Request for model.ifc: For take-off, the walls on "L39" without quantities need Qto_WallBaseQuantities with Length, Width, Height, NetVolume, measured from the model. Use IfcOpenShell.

First a look at what the model holds.

```python
import ifcopenshell
import ifcopenshell.util.element
import ifcopenshell.util.unit

model = ifcopenshell.open("model.ifc")
print(model.schema)
for unit_type in ("LENGTHUNIT", "AREAUNIT", "VOLUMEUNIT"):
    print(unit_type, ifcopenshell.util.unit.calculate_unit_scale(model, unit_type))
storey = next(s for s in model.by_type("IfcBuildingStorey") if s.Name == "L39")
walls = [e for e in ifcopenshell.util.element.get_decomposition(storey) if e.is_a("IfcWall")]
for e in sorted(walls, key=lambda e: e.id()):
    print(e.id(), e.is_a(), e.Name, list(ifcopenshell.util.element.get_psets(e, qtos_only=True)), sep=" | ")
```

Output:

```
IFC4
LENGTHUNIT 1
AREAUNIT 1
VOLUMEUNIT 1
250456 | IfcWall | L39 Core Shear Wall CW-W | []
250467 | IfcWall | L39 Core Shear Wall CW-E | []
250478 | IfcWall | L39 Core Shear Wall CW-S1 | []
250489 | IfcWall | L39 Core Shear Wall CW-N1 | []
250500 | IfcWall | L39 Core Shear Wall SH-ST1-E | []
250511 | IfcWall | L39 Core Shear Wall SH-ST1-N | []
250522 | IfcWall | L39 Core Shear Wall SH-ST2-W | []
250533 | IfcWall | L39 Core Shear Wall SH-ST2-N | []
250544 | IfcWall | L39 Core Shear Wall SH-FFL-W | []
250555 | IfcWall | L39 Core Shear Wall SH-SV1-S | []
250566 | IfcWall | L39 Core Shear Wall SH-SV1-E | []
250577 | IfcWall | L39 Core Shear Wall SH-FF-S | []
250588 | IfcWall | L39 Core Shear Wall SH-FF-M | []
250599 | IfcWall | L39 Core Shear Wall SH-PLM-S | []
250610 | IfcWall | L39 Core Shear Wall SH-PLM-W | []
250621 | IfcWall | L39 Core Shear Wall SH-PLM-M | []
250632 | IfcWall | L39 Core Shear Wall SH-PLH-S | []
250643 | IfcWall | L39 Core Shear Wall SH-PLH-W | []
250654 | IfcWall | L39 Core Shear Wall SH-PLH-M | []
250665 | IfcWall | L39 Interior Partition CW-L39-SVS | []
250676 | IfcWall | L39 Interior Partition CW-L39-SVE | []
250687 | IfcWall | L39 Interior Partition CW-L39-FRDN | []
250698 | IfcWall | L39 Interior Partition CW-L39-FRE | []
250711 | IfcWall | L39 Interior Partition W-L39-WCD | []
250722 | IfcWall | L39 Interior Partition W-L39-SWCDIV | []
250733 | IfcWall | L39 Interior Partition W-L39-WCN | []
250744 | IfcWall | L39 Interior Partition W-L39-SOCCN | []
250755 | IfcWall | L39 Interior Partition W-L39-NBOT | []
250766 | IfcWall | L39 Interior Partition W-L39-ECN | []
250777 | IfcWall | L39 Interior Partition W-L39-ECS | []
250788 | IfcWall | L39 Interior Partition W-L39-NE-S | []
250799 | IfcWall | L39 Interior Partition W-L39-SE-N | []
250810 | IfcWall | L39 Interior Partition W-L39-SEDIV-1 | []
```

```python
import ifcopenshell
import ifcopenshell.api.pset
import ifcopenshell.geom
import ifcopenshell.util.element
import ifcopenshell.util.shape
import ifcopenshell.util.unit

model = ifcopenshell.open("model.ifc")
unit_scale = ifcopenshell.util.unit.calculate_unit_scale(model)
volume_scale = ifcopenshell.util.unit.calculate_unit_scale(model, "VOLUMEUNIT")
settings = ifcopenshell.geom.settings()

storey = next(s for s in model.by_type("IfcBuildingStorey") if s.Name == "L39")
walls = [e for e in ifcopenshell.util.element.get_decomposition(storey) if e.is_a("IfcWall")]

for e in sorted(walls, key=lambda e: e.id()):
    if ifcopenshell.util.element.get_psets(e, qtos_only=True, should_inherit=False):
        continue
    # Geometry comes back in metres, in the element's own axes.
    shape = ifcopenshell.geom.create_shape(settings, e)
    values = {
        "Length": ifcopenshell.util.shape.get_x(shape.geometry) / unit_scale,
        "Width": ifcopenshell.util.shape.get_y(shape.geometry) / unit_scale,
        "Height": ifcopenshell.util.shape.get_z(shape.geometry) / unit_scale,
        "NetVolume": ifcopenshell.util.shape.get_volume(shape.geometry) / volume_scale,
    }
    qto = ifcopenshell.api.pset.add_qto(model, product=e, name="Qto_WallBaseQuantities")
    ifcopenshell.api.pset.edit_qto(model, qto=qto, properties=values)
    print(e.id(), {k: round(v, 3) for k, v in values.items()})

model.write("model_updated.ifc")
```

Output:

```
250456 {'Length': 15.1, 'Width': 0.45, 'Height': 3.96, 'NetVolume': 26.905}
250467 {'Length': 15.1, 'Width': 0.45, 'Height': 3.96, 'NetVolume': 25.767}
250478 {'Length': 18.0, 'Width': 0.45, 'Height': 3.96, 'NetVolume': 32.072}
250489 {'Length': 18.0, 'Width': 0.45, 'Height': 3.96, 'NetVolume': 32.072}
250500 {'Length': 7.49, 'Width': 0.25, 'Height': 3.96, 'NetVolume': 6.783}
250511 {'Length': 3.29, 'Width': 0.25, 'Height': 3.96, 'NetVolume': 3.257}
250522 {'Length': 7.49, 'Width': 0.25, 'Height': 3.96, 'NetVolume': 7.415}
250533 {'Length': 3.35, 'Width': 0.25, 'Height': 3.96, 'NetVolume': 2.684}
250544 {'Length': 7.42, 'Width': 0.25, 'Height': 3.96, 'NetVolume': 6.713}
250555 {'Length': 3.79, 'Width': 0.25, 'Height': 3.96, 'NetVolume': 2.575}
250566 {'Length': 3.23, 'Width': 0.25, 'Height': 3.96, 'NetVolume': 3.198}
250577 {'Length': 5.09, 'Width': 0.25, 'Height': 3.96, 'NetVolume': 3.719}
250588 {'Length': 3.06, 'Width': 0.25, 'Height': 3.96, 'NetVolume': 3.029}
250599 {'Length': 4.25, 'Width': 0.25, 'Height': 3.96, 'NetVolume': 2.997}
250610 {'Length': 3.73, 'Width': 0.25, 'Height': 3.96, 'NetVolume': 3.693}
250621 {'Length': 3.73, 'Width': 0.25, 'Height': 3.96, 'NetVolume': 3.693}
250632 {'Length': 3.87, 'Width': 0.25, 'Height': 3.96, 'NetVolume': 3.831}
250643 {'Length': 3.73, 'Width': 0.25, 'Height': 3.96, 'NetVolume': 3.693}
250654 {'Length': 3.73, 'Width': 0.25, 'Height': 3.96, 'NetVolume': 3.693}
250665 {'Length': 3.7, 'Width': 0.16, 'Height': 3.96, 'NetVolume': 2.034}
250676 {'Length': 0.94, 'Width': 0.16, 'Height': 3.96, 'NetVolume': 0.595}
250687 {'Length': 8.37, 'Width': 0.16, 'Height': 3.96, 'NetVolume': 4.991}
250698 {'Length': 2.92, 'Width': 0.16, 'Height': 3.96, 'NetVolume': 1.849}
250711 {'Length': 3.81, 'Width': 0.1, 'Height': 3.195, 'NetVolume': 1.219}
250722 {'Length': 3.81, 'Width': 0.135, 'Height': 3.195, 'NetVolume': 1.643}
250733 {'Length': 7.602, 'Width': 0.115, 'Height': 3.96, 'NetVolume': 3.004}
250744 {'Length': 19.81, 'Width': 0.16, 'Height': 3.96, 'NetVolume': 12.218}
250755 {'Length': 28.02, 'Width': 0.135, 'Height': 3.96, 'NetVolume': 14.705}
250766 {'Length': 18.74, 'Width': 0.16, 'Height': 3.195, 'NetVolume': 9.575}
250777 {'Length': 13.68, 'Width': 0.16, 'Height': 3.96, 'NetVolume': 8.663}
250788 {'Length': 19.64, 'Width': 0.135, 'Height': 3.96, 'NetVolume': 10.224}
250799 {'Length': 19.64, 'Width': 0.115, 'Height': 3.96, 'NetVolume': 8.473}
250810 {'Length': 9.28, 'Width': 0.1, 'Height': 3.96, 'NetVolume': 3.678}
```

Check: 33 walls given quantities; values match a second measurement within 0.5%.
